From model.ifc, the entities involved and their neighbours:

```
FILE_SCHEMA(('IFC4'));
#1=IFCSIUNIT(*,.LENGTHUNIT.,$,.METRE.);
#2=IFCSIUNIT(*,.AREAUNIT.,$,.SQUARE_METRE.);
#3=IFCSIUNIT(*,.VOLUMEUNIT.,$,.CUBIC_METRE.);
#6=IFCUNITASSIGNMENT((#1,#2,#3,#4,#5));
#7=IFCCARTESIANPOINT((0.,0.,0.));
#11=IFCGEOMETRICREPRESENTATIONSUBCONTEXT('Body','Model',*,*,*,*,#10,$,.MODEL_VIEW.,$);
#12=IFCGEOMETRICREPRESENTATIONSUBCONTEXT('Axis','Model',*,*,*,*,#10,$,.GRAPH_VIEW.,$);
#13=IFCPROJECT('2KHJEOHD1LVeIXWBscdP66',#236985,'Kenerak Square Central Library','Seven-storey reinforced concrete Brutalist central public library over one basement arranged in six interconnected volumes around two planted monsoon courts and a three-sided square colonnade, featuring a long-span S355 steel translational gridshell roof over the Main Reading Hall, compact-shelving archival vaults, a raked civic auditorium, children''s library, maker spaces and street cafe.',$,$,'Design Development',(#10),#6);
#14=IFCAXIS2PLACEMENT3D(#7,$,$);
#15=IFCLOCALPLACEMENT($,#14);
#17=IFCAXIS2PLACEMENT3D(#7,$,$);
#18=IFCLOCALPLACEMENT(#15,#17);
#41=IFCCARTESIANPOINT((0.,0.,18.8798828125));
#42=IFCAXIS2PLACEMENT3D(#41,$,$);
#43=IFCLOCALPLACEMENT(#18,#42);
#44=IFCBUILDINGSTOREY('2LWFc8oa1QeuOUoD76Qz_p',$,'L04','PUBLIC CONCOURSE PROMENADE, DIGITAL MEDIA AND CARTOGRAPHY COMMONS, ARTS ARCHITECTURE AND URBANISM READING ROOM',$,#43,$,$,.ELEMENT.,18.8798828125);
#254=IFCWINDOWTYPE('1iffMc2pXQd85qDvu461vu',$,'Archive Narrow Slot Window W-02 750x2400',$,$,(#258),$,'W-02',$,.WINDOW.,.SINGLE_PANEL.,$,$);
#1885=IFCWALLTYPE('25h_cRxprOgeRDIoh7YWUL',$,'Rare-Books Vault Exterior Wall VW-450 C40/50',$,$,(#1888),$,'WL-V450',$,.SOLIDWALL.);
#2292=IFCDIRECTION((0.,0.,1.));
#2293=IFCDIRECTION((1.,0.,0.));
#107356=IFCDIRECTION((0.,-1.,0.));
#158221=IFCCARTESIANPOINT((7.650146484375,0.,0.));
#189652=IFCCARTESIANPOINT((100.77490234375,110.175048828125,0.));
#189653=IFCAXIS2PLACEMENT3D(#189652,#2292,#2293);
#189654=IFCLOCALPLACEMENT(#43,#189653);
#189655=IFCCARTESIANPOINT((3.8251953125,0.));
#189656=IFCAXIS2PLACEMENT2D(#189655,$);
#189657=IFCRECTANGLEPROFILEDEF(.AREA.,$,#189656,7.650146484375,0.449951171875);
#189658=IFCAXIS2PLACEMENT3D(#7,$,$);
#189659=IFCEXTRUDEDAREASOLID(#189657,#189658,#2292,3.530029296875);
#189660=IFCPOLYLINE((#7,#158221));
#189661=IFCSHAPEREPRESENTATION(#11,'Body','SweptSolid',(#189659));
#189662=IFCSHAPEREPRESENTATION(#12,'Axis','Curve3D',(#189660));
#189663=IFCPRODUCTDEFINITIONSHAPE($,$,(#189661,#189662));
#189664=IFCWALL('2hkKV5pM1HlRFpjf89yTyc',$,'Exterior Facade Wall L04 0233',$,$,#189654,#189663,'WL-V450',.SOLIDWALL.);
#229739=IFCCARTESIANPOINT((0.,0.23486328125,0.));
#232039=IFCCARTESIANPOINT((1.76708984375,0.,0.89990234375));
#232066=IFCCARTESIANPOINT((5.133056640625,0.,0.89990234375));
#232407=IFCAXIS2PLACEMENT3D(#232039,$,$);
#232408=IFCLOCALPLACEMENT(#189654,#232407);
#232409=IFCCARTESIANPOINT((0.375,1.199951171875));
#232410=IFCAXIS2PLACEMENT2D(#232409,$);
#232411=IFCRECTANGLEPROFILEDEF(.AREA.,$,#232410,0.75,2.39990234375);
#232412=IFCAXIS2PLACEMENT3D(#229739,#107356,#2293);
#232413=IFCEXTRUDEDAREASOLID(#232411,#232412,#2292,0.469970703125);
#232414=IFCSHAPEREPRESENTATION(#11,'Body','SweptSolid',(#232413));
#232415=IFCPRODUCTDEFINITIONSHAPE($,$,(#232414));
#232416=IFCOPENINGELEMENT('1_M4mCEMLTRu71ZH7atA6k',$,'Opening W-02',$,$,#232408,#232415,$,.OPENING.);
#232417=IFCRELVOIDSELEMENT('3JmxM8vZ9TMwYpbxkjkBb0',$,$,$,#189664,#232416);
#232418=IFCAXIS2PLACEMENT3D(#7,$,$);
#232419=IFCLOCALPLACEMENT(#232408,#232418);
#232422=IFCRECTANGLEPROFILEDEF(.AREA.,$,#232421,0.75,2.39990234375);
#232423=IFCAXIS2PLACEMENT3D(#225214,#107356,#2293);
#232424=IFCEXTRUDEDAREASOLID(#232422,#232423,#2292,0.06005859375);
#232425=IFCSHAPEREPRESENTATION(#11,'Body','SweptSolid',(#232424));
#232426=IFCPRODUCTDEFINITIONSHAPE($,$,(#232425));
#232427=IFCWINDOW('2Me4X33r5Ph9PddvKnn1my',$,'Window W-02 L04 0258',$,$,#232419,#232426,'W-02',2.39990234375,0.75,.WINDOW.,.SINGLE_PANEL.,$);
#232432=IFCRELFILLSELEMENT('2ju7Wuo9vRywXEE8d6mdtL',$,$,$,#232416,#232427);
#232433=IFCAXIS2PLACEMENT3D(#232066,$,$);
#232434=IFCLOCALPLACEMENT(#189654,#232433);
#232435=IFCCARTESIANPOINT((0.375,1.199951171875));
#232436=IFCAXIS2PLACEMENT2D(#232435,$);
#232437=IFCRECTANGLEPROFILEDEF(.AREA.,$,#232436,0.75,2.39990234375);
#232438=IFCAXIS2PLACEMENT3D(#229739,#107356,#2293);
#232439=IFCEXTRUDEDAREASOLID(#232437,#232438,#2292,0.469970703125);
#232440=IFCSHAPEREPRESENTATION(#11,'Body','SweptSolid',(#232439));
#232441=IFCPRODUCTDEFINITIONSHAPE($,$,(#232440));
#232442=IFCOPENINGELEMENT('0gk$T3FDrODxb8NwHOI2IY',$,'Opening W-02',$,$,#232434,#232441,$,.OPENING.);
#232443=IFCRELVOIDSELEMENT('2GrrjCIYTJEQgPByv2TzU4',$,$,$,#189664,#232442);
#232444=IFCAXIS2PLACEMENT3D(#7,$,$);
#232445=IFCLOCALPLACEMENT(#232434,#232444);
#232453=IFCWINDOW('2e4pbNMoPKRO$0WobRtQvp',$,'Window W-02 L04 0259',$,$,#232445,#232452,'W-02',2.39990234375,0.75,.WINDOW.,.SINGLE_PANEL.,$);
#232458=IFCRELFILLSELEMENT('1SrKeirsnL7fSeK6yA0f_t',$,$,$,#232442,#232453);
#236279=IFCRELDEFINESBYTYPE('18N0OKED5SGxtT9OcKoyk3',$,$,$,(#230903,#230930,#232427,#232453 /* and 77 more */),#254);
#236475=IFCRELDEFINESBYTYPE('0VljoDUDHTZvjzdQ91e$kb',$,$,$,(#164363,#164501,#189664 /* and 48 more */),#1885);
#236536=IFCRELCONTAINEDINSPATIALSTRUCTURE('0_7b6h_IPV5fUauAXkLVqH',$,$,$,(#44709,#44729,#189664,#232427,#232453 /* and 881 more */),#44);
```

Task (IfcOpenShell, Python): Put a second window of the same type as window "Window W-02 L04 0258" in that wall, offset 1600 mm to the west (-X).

```python
import ifcopenshell
import ifcopenshell.api.feature
import ifcopenshell.api.geometry
import ifcopenshell.api.root
import ifcopenshell.geom
import ifcopenshell.util.element
import ifcopenshell.util.placement
import ifcopenshell.util.shape

model = ifcopenshell.open("model.ifc")
settings = ifcopenshell.geom.settings()


def volume(element):
    """Net volume in cubic metres, openings subtracted."""
    shape = ifcopenshell.geom.create_shape(settings, element)
    return ifcopenshell.util.shape.get_volume(shape.geometry)


window = model.by_guid("2Me4X33r5Ph9PddvKnn1my")
opening = window.FillsVoids[0].RelatingOpeningElement
wall = opening.VoidsElements[0].RelatingBuildingElement
before = volume(wall)
shift = ifcopenshell.util.placement.get_local_placement(wall.ObjectPlacement)[:3, 0] * -1.6

# copy_class copies the void relationship, type, container and properties, but no geometry.
new_opening = ifcopenshell.api.root.copy_class(model, product=opening)
new_opening.Representation = ifcopenshell.util.element.copy_deep(
    model, opening.Representation, exclude=["IfcGeometricRepresentationContext", "IfcRepresentationMap"]
)
new_window = ifcopenshell.api.root.copy_class(model, product=window)
new_window.Representation = ifcopenshell.util.element.copy_deep(
    model, window.Representation, exclude=["IfcGeometricRepresentationContext", "IfcRepresentationMap"]
)
new_window.Tag = None
ifcopenshell.api.feature.add_filling(model, opening=new_opening, element=new_window)

for old, new in ((opening, new_opening), (window, new_window)):
    matrix = ifcopenshell.util.placement.get_local_placement(old.ObjectPlacement)
    matrix[:3, 3] += shift
    ifcopenshell.api.geometry.edit_object_placement(model, product=new, matrix=matrix, is_si=False)

after = volume(wall)

print(f"wall volume {before:.3f} -> {after:.3f} m3")

model.write("model_updated.ifc")
```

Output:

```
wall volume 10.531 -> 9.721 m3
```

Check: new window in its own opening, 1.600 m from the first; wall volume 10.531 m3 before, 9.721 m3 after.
